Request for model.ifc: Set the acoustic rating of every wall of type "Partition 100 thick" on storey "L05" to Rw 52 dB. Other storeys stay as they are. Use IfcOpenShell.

First a look at what the model holds.

```python
import ifcopenshell
import ifcopenshell.util.element

model = ifcopenshell.open("model.ifc")
print(model.schema)
storey = next(s for s in model.by_type("IfcBuildingStorey") if s.Name == "L05")
walls = [e for e in ifcopenshell.util.element.get_decomposition(storey) if e.is_a("IfcWall")]
seen = {}
for e in walls:
    element_type = ifcopenshell.util.element.get_type(e)
    key = (element_type.Name if element_type != e and element_type else None, ifcopenshell.util.element.get_pset(e, "Pset_WallCommon", "AcousticRating"))
    seen[key] = seen.get(key, 0) + 1
for (name, value), count in sorted(seen.items(), key=str):
    print(count, "x", name, "|", value)
```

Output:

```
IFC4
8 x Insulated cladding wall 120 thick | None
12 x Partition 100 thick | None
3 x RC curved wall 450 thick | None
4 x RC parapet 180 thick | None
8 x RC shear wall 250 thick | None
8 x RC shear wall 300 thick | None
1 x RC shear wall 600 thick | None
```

```python
import ifcopenshell
import ifcopenshell.api.pset
import ifcopenshell.util.element

model = ifcopenshell.open("model.ifc")

storey = next(s for s in model.by_type("IfcBuildingStorey") if s.Name == "L05")
walls = [e for e in ifcopenshell.util.element.get_decomposition(storey) if e.is_a("IfcWall")]

count = 0
for e in walls:
    element_type = ifcopenshell.util.element.get_type(e)
    if element_type in (None, e) or element_type.Name != "Partition 100 thick":
        continue
    # add_pset returns the element's existing set when there is one.
    pset = ifcopenshell.api.pset.add_pset(model, product=e, name="Pset_WallCommon")
    ifcopenshell.api.pset.edit_pset(model, pset=pset, properties={"AcousticRating": "Rw 52 dB"})
    count += 1

print(count, "walls updated")

model.write("model_edited.ifc")
```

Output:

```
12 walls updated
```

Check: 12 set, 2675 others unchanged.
